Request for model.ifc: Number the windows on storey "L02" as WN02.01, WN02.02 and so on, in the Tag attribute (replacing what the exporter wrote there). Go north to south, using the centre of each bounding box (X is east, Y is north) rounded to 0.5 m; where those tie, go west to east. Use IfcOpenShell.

First a look at what the model holds.

```python
import ifcopenshell
import ifcopenshell.util.element
import ifcopenshell.util.placement

model = ifcopenshell.open("model.ifc")
print(model.schema)
storey = next(s for s in model.by_type("IfcBuildingStorey") if s.Name == "L02")
windows = [e for e in ifcopenshell.util.element.get_decomposition(storey) if e.is_a("IfcWindow")]
for e in sorted(windows, key=lambda e: e.id()):
    origin = ifcopenshell.util.placement.get_local_placement(e.ObjectPlacement)[:3, 3]
    print(e.id(), e.Tag, e.Name, origin.round(2) + 0.0, sep=" | ")
```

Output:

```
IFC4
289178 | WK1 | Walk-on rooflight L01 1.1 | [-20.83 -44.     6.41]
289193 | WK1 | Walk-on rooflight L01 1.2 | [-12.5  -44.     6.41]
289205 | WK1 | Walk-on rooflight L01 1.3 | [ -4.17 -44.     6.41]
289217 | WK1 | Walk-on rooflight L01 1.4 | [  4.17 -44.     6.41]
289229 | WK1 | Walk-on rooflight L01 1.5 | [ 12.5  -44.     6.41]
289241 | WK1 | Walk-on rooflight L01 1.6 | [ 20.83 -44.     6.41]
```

```python
import ifcopenshell
import ifcopenshell.geom
import ifcopenshell.util.element
import ifcopenshell.util.shape

model = ifcopenshell.open("model.ifc")
settings = ifcopenshell.geom.settings()
settings.set("use-world-coords", True)


def centre(element):
    shape = ifcopenshell.geom.create_shape(settings, element)
    return ifcopenshell.util.shape.get_bbox_centroid(shape.geometry)


storey = next(s for s in model.by_type("IfcBuildingStorey") if s.Name == "L02")
windows = [e for e in ifcopenshell.util.element.get_decomposition(storey) if e.is_a("IfcWindow")]

# Insertion points can sit at a corner or the storey origin, so sort by the geometry (in metres).
centres = {e: centre(e) for e in windows}
windows.sort(key=lambda e: (-round(centres[e][1] / 0.5), centres[e][0]))

for i, e in enumerate(windows, start=1):
    number = f"WN02.{i:02d}"
    e.Tag = number
    print(e.id(), number)

model.write("model_v2.ifc")
```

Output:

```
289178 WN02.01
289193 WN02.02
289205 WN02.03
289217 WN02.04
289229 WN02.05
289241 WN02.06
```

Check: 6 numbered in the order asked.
